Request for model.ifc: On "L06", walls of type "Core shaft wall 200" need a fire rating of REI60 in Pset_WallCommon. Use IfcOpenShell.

First a look at what the model holds.

```python
import ifcopenshell
import ifcopenshell.util.element

model = ifcopenshell.open("model.ifc")
print(model.schema)
storey = next(s for s in model.by_type("IfcBuildingStorey") if s.Name == "L06")
walls = [e for e in ifcopenshell.util.element.get_decomposition(storey) if e.is_a("IfcWall")]
seen = {}
for e in walls:
    element_type = ifcopenshell.util.element.get_type(e)
    key = (element_type.Name if element_type != e and element_type else None, ifcopenshell.util.element.get_pset(e, "Pset_WallCommon", "FireRating"))
    seen[key] = seen.get(key, 0) + 1
for (name, value), count in sorted(seen.items(), key=str):
    print(count, "x", name, "|", value)
```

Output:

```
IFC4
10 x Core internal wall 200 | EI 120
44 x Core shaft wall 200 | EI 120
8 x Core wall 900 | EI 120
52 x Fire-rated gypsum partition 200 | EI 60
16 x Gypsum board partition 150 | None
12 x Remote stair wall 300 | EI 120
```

```python
import ifcopenshell
import ifcopenshell.api.pset
import ifcopenshell.util.element

model = ifcopenshell.open("model.ifc")

storey = next(s for s in model.by_type("IfcBuildingStorey") if s.Name == "L06")
walls = [e for e in ifcopenshell.util.element.get_decomposition(storey) if e.is_a("IfcWall")]

count = 0
for e in walls:
    element_type = ifcopenshell.util.element.get_type(e)
    if element_type in (None, e) or element_type.Name != "Core shaft wall 200":
        continue
    found = ifcopenshell.util.element.get_pset(e, "Pset_WallCommon", should_inherit=False)
    if found:
        pset = model.by_id(found["id"])
        if len(ifcopenshell.util.element.get_elements_by_pset(pset)) > 1:
            pset = ifcopenshell.api.pset.unshare_pset(model, products=[e], pset=pset)[0]
    else:
        pset = ifcopenshell.api.pset.add_pset(model, product=e, name="Pset_WallCommon")
    ifcopenshell.api.pset.edit_pset(model, pset=pset, properties={"FireRating": "REI60"})
    count += 1

print(count, "walls updated")

model.write("model-out.ifc")
```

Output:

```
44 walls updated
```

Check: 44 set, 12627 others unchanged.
